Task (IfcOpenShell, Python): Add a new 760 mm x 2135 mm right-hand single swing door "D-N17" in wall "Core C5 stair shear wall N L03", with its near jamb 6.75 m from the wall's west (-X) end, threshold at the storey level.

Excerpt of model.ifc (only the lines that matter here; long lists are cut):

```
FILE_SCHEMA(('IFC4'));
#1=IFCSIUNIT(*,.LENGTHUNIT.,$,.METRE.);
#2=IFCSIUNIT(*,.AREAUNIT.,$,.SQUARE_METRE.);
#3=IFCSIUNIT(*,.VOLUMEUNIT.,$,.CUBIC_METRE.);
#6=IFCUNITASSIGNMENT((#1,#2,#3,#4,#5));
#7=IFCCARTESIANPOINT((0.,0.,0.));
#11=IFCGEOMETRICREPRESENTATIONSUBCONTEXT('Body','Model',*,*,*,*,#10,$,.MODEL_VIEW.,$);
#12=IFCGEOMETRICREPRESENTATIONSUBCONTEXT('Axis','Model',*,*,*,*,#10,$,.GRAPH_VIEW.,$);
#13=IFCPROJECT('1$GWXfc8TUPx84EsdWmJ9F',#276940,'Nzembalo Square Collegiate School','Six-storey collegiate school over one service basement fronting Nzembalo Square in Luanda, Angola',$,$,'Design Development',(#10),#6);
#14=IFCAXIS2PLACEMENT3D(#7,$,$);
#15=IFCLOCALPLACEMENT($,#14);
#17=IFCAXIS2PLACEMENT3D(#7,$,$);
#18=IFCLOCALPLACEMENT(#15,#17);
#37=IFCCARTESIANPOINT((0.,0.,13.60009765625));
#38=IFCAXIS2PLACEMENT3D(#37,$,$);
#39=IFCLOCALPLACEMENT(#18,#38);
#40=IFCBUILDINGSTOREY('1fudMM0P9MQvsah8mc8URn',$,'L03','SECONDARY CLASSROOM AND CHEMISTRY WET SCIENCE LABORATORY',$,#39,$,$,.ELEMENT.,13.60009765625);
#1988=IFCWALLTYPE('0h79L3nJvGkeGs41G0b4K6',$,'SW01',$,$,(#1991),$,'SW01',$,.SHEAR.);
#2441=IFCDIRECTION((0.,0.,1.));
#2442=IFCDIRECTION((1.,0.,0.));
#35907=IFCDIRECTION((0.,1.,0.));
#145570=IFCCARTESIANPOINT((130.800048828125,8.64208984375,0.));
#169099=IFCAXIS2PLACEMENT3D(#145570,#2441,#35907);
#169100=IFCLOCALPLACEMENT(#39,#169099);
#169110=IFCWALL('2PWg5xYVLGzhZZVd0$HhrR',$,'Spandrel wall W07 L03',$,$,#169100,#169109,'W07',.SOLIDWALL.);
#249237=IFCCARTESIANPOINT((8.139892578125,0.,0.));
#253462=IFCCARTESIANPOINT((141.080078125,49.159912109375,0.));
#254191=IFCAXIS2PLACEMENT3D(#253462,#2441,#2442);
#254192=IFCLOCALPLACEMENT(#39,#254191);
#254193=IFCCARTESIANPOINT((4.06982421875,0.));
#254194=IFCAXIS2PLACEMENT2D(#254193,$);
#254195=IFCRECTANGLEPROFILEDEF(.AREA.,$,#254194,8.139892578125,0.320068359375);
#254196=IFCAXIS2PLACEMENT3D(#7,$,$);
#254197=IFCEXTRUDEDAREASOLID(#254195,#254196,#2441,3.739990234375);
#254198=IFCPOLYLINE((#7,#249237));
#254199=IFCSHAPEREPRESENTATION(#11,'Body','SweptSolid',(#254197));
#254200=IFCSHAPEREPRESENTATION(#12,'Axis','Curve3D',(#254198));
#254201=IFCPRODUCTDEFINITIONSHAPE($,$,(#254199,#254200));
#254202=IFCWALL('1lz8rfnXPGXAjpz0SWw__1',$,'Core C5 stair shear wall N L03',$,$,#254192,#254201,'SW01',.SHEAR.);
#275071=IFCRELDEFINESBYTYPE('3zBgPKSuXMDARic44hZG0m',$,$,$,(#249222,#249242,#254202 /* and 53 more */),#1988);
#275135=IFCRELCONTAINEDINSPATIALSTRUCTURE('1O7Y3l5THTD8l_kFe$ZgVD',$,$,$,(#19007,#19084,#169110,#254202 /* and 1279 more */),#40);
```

```python
import numpy as np
import ifcopenshell
import ifcopenshell.api.feature
import ifcopenshell.api.geometry
import ifcopenshell.api.root
import ifcopenshell.api.spatial
import ifcopenshell.geom
import ifcopenshell.util.element
import ifcopenshell.util.placement
import ifcopenshell.util.representation
import ifcopenshell.util.shape
import ifcopenshell.util.unit

model = ifcopenshell.open("model.ifc")
unit_scale = ifcopenshell.util.unit.calculate_unit_scale(model)
settings = ifcopenshell.geom.settings()


def volume(element):
    """Net volume in cubic metres, openings subtracted."""
    shape = ifcopenshell.geom.create_shape(settings, element)
    return ifcopenshell.util.shape.get_volume(shape.geometry)


wall = model.by_guid("1lz8rfnXPGXAjpz0SWw__1")
storey = ifcopenshell.util.element.get_container(wall, ifc_class="IfcBuildingStorey")
context = ifcopenshell.util.representation.get_context(model, "Model", "Body", "MODEL_VIEW")
before = volume(wall)

width, height, from_end, sill = 0.76, 2.135, 6.75, 0.0  # metres

# The wall runs along its own X axis, and the end named is its -X end.
wall_shape = ifcopenshell.geom.create_shape(settings, wall)
x, y, z = ifcopenshell.util.shape.get_vertices(wall_shape.geometry).T
start = x.min() + from_end
face, thickness = float(y.min()), float(y.max() - y.min())
wall_matrix = ifcopenshell.util.placement.get_local_placement(wall.ObjectPlacement)
level = ifcopenshell.util.placement.get_local_placement(storey.ObjectPlacement)[2, 3]


def in_wall(x, y):
    """Placement at x, y metres in the wall's axes, at sill height."""
    matrix = wall_matrix.copy()
    matrix[:, 3] = wall_matrix @ np.array([x / unit_scale, y / unit_scale, 0.0, 1.0])
    matrix[2, 3] = level + sill / unit_scale
    return matrix


# Opening: a box that overshoots both wall faces by 50 mm.
opening = ifcopenshell.api.root.create_entity(model, ifc_class="IfcOpeningElement", predefined_type="OPENING")
box = ifcopenshell.api.geometry.add_wall_representation(
    model, context=context, length=width, height=height, thickness=thickness + 0.1
)
ifcopenshell.api.geometry.assign_representation(model, product=opening, representation=box)
ifcopenshell.api.geometry.edit_object_placement(model, product=opening, matrix=in_wall(start, face - 0.05), is_si=False)
ifcopenshell.api.feature.add_feature(model, feature=opening, element=wall)

door = ifcopenshell.api.root.create_entity(model, ifc_class="IfcDoor", name="D-N17", predefined_type="DOOR")
door.OverallWidth, door.OverallHeight = width / unit_scale, height / unit_scale
door.OperationType = "SINGLE_SWING_RIGHT"
body = ifcopenshell.api.geometry.add_door_representation(
    model,
    context=context,
    overall_width=door.OverallWidth,
    overall_height=door.OverallHeight,
    operation_type="SINGLE_SWING_RIGHT",
    lining_properties={"LiningDepth": thickness / unit_scale, "ThresholdDepth": thickness / unit_scale},
)
ifcopenshell.api.geometry.assign_representation(model, product=door, representation=body)
ifcopenshell.api.spatial.assign_container(model, products=[door], relating_structure=storey)
ifcopenshell.api.feature.add_filling(model, opening=opening, element=door)

# The lining spans the wall, so the door starts at the wall face.
ifcopenshell.api.geometry.edit_object_placement(model, product=door, matrix=in_wall(start, face), is_si=False)

after = volume(wall)

print(f"wall volume {before:.3f} -> {after:.3f} m3")

model.write("model_edited.ifc")
```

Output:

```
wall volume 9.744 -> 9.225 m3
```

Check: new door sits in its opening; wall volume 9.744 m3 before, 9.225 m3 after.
